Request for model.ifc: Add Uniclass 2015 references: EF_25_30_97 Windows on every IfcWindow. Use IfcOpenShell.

First a look at what the model holds.

```python
import ifcopenshell

model = ifcopenshell.open("model.ifc")
print(model.schema)
print("classifications:", [c.Name for c in model.by_type("IfcClassification")])
for ifc_class in ("IfcDoor", "IfcRoof", "IfcStair", "IfcWall", "IfcWindow"):
    print(ifc_class, len(model.by_type(ifc_class)))
```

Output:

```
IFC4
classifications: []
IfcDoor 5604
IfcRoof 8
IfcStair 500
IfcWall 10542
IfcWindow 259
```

```python
import ifcopenshell
import ifcopenshell.api.classification

model = ifcopenshell.open("model.ifc")

system = ifcopenshell.api.classification.add_classification(model, classification="Uniclass 2015")

codes = {
    "IfcWindow": ("EF_25_30_97", "Windows"),
}
for ifc_class, (code, name) in codes.items():
    products = model.by_type(ifc_class)
    ifcopenshell.api.classification.add_reference(
        model, products=products, classification=system, identification=code, name=name
    )
    print(code, len(products))

model.write("model_updated.ifc")
```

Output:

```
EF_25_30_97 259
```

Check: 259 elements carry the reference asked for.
